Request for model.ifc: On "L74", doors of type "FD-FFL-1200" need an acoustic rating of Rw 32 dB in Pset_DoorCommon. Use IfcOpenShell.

First a look at what the model holds.

```python
import ifcopenshell
import ifcopenshell.util.element

model = ifcopenshell.open("model.ifc")
print(model.schema)
storey = next(s for s in model.by_type("IfcBuildingStorey") if s.Name == "L74")
doors = [e for e in ifcopenshell.util.element.get_decomposition(storey) if e.is_a("IfcDoor")]
seen = {}
for e in doors:
    element_type = ifcopenshell.util.element.get_type(e)
    key = (element_type.Name if element_type != e and element_type else None, ifcopenshell.util.element.get_pset(e, "Pset_DoorCommon", "AcousticRating"))
    seen[key] = seen.get(key, 0) + 1
for (name, value), count in sorted(seen.items(), key=str):
    print(count, "x", name, "|", value)
```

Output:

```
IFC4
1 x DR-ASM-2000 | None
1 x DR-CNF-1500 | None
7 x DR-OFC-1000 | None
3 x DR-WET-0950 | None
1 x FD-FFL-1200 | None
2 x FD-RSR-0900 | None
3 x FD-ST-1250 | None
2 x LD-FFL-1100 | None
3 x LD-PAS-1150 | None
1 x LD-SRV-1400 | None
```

```python
import ifcopenshell
import ifcopenshell.api.pset
import ifcopenshell.util.element

model = ifcopenshell.open("model.ifc")

storey = next(s for s in model.by_type("IfcBuildingStorey") if s.Name == "L74")
doors = [e for e in ifcopenshell.util.element.get_decomposition(storey) if e.is_a("IfcDoor")]

count = 0
for e in doors:
    element_type = ifcopenshell.util.element.get_type(e)
    if element_type in (None, e) or element_type.Name != "FD-FFL-1200":
        continue
    # add_pset returns the element's existing set when there is one.
    pset = ifcopenshell.api.pset.add_pset(model, product=e, name="Pset_DoorCommon")
    ifcopenshell.api.pset.edit_pset(model, pset=pset, properties={"AcousticRating": "Rw 32 dB"})
    count += 1

print(count, "doors updated")

model.write("model-out.ifc")
```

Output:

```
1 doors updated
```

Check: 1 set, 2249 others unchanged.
